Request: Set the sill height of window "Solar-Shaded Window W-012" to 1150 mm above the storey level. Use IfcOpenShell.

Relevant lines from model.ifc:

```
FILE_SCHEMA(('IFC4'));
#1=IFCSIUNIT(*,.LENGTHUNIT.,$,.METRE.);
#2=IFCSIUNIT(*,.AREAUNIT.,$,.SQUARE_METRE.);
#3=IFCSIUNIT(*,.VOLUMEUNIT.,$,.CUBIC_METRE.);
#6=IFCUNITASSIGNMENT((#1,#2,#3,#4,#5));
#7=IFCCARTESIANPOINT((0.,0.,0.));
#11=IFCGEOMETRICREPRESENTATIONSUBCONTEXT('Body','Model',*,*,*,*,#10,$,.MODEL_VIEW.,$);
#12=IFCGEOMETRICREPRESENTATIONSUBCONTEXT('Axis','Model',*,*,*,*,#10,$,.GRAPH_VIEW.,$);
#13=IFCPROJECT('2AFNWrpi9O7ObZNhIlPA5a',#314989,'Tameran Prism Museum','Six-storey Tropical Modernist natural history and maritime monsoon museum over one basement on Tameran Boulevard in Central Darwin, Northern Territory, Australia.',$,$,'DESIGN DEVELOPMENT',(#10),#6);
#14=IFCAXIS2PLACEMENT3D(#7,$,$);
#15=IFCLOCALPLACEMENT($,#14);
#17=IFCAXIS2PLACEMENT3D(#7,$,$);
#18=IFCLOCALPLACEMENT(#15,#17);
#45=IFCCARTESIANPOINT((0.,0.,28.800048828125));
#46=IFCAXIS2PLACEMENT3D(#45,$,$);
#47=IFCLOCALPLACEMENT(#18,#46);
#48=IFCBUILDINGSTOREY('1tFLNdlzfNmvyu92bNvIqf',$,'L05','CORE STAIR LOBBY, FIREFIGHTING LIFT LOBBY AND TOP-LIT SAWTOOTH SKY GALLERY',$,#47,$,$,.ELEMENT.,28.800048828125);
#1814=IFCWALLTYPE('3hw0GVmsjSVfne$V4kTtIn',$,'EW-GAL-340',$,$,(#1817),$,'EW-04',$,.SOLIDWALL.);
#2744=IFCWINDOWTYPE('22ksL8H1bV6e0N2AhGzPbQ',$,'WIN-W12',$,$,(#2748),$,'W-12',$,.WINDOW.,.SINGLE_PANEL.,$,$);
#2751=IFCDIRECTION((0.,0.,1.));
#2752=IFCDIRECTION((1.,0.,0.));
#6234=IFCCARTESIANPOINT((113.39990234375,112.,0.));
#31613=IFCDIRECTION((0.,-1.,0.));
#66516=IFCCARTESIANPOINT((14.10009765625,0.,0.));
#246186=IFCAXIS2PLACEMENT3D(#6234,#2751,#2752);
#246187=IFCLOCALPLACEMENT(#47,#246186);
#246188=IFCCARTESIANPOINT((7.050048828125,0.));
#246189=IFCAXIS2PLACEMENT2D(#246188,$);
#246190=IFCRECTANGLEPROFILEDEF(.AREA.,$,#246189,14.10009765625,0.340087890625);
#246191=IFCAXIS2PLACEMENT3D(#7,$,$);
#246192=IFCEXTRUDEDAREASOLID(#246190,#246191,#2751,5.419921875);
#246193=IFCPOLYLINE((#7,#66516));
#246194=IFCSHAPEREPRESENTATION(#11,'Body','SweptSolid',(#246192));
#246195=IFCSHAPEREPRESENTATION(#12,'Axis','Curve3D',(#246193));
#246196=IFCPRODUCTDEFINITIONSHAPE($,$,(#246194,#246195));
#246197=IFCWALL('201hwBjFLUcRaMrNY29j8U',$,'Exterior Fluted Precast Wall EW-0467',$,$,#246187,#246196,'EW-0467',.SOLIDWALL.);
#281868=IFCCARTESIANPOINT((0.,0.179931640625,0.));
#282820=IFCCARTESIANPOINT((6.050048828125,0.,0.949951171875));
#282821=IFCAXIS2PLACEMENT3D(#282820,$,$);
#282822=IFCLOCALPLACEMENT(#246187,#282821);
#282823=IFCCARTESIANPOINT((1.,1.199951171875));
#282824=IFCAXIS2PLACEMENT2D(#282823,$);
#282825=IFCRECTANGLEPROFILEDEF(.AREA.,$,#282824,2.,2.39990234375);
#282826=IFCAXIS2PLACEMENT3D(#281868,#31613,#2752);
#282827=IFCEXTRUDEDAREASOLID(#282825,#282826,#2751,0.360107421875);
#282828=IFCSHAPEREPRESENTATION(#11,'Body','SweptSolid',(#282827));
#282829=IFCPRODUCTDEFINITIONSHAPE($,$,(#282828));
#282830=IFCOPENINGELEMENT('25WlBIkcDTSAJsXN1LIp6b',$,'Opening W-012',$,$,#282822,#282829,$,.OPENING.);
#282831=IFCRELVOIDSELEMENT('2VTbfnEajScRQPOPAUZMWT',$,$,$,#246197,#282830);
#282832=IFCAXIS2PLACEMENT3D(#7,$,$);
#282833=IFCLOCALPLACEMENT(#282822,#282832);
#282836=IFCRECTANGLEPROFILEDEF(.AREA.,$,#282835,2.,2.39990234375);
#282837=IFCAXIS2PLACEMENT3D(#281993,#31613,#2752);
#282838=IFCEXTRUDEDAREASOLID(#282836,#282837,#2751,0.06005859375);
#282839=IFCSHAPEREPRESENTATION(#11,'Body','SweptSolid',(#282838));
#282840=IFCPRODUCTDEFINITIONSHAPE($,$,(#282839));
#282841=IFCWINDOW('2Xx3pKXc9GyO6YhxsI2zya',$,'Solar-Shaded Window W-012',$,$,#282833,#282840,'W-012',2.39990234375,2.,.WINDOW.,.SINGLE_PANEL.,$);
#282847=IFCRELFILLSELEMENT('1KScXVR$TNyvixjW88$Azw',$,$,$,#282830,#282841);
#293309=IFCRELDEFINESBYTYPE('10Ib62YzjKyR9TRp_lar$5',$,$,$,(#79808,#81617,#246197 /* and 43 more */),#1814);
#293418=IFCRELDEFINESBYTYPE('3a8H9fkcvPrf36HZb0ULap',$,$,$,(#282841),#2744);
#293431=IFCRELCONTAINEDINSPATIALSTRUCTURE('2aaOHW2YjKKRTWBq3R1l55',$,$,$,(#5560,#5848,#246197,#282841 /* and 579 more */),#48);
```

```python
import numpy as np
import ifcopenshell
import ifcopenshell.api.geometry
import ifcopenshell.geom
import ifcopenshell.util.element
import ifcopenshell.util.placement
import ifcopenshell.util.shape
import ifcopenshell.util.unit

model = ifcopenshell.open("model.ifc")
unit_scale = ifcopenshell.util.unit.calculate_unit_scale(model)

window = model.by_guid("2Xx3pKXc9GyO6YhxsI2zya")
opening = window.FillsVoids[0].RelatingOpeningElement
storey = ifcopenshell.util.element.get_container(window, ifc_class="IfcBuildingStorey")
level = ifcopenshell.util.placement.get_local_placement(storey.ObjectPlacement)[2, 3]

# The opening's origin need not be at the sill, so measure its lowest point.
shape = ifcopenshell.geom.create_shape(ifcopenshell.geom.settings(), opening)
bottom = ifcopenshell.util.shape.get_shape_bottom_elevation(shape, shape.geometry) / unit_scale
dz = level + 1.15 / unit_scale - bottom

shift = np.array([0.0, 0.0, dz])
# The window is placed relative to its opening, so it follows when the opening moves.
matrix = ifcopenshell.util.placement.get_local_placement(opening.ObjectPlacement)
matrix[:3, 3] += shift
ifcopenshell.api.geometry.edit_object_placement(
    model, product=opening, matrix=matrix, is_si=False, should_transform_children=True
)

print(f"moved by {dz * unit_scale:+.3f} m")

model.write("model_rev.ifc")
```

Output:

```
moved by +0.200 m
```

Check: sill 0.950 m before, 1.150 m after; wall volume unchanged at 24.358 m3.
